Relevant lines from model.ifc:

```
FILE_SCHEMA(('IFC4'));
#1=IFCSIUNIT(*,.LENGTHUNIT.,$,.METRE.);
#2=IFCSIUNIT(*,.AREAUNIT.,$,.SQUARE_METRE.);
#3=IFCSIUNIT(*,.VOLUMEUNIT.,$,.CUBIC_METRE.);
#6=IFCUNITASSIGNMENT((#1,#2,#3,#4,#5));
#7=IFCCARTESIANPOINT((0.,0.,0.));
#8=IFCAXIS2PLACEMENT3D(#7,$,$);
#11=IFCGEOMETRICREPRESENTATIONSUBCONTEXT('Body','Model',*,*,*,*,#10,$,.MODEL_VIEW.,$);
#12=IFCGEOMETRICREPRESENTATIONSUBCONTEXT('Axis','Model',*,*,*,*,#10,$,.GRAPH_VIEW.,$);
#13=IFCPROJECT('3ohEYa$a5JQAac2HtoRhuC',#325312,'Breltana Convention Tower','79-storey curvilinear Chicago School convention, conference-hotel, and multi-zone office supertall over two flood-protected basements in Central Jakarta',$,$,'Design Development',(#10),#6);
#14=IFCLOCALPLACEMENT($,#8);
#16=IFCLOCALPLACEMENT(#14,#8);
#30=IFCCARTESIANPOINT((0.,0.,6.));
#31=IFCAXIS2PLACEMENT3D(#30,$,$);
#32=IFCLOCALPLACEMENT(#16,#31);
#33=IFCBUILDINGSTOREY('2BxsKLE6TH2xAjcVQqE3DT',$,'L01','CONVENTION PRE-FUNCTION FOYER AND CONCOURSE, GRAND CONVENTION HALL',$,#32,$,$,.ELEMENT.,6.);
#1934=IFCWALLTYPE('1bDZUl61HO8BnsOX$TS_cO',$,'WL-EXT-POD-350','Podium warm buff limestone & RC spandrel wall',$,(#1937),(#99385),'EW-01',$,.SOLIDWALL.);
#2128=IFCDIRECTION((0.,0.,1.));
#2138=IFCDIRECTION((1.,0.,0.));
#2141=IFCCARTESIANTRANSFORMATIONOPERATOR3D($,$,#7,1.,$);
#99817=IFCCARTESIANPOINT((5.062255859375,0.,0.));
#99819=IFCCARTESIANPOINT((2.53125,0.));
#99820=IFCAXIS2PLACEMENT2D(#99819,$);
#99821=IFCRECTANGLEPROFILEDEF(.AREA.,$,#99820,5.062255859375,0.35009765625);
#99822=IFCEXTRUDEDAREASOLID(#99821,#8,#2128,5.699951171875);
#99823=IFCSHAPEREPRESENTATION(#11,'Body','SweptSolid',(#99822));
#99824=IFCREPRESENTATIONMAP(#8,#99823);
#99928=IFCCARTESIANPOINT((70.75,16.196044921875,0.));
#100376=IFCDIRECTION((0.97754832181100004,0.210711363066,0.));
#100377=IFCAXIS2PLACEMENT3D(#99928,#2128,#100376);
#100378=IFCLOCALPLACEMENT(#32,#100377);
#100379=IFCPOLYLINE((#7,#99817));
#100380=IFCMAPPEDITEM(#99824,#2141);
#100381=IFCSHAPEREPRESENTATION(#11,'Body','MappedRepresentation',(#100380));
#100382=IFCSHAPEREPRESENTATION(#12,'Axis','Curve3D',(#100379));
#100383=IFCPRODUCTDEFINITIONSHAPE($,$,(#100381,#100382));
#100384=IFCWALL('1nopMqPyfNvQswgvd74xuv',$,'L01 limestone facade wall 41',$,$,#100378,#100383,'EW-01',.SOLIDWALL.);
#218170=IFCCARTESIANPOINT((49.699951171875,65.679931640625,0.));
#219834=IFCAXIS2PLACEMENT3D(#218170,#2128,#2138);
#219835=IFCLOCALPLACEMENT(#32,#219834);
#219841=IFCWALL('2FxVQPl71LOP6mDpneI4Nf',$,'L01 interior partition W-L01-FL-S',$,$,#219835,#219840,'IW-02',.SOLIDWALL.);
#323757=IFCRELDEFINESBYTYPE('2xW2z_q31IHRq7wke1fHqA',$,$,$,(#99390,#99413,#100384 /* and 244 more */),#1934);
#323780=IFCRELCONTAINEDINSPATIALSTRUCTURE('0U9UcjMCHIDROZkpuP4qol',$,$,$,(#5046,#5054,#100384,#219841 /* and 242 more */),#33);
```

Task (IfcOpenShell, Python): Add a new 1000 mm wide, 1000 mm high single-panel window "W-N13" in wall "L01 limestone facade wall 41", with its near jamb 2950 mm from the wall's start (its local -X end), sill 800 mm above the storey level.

```python
import numpy as np
import ifcopenshell
import ifcopenshell.api.feature
import ifcopenshell.api.geometry
import ifcopenshell.api.root
import ifcopenshell.api.spatial
import ifcopenshell.geom
import ifcopenshell.util.element
import ifcopenshell.util.placement
import ifcopenshell.util.representation
import ifcopenshell.util.shape
import ifcopenshell.util.unit

model = ifcopenshell.open("model.ifc")
unit_scale = ifcopenshell.util.unit.calculate_unit_scale(model)
settings = ifcopenshell.geom.settings()


def volume(element):
    """Net volume in cubic metres, openings subtracted."""
    shape = ifcopenshell.geom.create_shape(settings, element)
    return ifcopenshell.util.shape.get_volume(shape.geometry)


wall = model.by_guid("1nopMqPyfNvQswgvd74xuv")
storey = ifcopenshell.util.element.get_container(wall, ifc_class="IfcBuildingStorey")
context = ifcopenshell.util.representation.get_context(model, "Model", "Body", "MODEL_VIEW")
before = volume(wall)

width, height, from_end, sill = 1, 1, 2.95, 0.8  # metres

# The wall runs along its own X axis, and the end named is its -X end.
wall_shape = ifcopenshell.geom.create_shape(settings, wall)
x, y, z = ifcopenshell.util.shape.get_vertices(wall_shape.geometry).T
start = x.min() + from_end
face, thickness = float(y.min()), float(y.max() - y.min())
wall_matrix = ifcopenshell.util.placement.get_local_placement(wall.ObjectPlacement)
level = ifcopenshell.util.placement.get_local_placement(storey.ObjectPlacement)[2, 3]


def in_wall(x, y):
    """Placement at x, y metres in the wall's axes, at sill height."""
    matrix = wall_matrix.copy()
    matrix[:, 3] = wall_matrix @ np.array([x / unit_scale, y / unit_scale, 0.0, 1.0])
    matrix[2, 3] = level + sill / unit_scale
    return matrix


# Opening: a box that overshoots both wall faces by 50 mm.
opening = ifcopenshell.api.root.create_entity(model, ifc_class="IfcOpeningElement", predefined_type="OPENING")
box = ifcopenshell.api.geometry.add_wall_representation(
    model, context=context, length=width, height=height, thickness=thickness + 0.1
)
ifcopenshell.api.geometry.assign_representation(model, product=opening, representation=box)
ifcopenshell.api.geometry.edit_object_placement(model, product=opening, matrix=in_wall(start, face - 0.05), is_si=False)
ifcopenshell.api.feature.add_feature(model, feature=opening, element=wall)

window = ifcopenshell.api.root.create_entity(model, ifc_class="IfcWindow", name="W-N13", predefined_type="WINDOW")
window.OverallWidth, window.OverallHeight = width / unit_scale, height / unit_scale
window.PartitioningType = "SINGLE_PANEL"
body = ifcopenshell.api.geometry.add_window_representation(
    model,
    context=context,
    overall_width=window.OverallWidth,
    overall_height=window.OverallHeight,
    partition_type="SINGLE_PANEL",
)
ifcopenshell.api.geometry.assign_representation(model, product=window, representation=body)
ifcopenshell.api.spatial.assign_container(model, products=[window], relating_structure=storey)
ifcopenshell.api.feature.add_filling(model, opening=opening, element=window)

# Centre the window in the wall's thickness.
ifcopenshell.api.geometry.edit_object_placement(model, product=window, matrix=in_wall(start, face), is_si=False)
window_shape = ifcopenshell.geom.create_shape(settings, window)
depth = ifcopenshell.util.shape.get_vertices(window_shape.geometry)[:, 1]
offset = face + thickness / 2 - (depth.min() + depth.max()) / 2
ifcopenshell.api.geometry.edit_object_placement(model, product=window, matrix=in_wall(start, offset), is_si=False)

after = volume(wall)

print(f"wall volume {before:.3f} -> {after:.3f} m3")

model.write("model_v2.ifc")
```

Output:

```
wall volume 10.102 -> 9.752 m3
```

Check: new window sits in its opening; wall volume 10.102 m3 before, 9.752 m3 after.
